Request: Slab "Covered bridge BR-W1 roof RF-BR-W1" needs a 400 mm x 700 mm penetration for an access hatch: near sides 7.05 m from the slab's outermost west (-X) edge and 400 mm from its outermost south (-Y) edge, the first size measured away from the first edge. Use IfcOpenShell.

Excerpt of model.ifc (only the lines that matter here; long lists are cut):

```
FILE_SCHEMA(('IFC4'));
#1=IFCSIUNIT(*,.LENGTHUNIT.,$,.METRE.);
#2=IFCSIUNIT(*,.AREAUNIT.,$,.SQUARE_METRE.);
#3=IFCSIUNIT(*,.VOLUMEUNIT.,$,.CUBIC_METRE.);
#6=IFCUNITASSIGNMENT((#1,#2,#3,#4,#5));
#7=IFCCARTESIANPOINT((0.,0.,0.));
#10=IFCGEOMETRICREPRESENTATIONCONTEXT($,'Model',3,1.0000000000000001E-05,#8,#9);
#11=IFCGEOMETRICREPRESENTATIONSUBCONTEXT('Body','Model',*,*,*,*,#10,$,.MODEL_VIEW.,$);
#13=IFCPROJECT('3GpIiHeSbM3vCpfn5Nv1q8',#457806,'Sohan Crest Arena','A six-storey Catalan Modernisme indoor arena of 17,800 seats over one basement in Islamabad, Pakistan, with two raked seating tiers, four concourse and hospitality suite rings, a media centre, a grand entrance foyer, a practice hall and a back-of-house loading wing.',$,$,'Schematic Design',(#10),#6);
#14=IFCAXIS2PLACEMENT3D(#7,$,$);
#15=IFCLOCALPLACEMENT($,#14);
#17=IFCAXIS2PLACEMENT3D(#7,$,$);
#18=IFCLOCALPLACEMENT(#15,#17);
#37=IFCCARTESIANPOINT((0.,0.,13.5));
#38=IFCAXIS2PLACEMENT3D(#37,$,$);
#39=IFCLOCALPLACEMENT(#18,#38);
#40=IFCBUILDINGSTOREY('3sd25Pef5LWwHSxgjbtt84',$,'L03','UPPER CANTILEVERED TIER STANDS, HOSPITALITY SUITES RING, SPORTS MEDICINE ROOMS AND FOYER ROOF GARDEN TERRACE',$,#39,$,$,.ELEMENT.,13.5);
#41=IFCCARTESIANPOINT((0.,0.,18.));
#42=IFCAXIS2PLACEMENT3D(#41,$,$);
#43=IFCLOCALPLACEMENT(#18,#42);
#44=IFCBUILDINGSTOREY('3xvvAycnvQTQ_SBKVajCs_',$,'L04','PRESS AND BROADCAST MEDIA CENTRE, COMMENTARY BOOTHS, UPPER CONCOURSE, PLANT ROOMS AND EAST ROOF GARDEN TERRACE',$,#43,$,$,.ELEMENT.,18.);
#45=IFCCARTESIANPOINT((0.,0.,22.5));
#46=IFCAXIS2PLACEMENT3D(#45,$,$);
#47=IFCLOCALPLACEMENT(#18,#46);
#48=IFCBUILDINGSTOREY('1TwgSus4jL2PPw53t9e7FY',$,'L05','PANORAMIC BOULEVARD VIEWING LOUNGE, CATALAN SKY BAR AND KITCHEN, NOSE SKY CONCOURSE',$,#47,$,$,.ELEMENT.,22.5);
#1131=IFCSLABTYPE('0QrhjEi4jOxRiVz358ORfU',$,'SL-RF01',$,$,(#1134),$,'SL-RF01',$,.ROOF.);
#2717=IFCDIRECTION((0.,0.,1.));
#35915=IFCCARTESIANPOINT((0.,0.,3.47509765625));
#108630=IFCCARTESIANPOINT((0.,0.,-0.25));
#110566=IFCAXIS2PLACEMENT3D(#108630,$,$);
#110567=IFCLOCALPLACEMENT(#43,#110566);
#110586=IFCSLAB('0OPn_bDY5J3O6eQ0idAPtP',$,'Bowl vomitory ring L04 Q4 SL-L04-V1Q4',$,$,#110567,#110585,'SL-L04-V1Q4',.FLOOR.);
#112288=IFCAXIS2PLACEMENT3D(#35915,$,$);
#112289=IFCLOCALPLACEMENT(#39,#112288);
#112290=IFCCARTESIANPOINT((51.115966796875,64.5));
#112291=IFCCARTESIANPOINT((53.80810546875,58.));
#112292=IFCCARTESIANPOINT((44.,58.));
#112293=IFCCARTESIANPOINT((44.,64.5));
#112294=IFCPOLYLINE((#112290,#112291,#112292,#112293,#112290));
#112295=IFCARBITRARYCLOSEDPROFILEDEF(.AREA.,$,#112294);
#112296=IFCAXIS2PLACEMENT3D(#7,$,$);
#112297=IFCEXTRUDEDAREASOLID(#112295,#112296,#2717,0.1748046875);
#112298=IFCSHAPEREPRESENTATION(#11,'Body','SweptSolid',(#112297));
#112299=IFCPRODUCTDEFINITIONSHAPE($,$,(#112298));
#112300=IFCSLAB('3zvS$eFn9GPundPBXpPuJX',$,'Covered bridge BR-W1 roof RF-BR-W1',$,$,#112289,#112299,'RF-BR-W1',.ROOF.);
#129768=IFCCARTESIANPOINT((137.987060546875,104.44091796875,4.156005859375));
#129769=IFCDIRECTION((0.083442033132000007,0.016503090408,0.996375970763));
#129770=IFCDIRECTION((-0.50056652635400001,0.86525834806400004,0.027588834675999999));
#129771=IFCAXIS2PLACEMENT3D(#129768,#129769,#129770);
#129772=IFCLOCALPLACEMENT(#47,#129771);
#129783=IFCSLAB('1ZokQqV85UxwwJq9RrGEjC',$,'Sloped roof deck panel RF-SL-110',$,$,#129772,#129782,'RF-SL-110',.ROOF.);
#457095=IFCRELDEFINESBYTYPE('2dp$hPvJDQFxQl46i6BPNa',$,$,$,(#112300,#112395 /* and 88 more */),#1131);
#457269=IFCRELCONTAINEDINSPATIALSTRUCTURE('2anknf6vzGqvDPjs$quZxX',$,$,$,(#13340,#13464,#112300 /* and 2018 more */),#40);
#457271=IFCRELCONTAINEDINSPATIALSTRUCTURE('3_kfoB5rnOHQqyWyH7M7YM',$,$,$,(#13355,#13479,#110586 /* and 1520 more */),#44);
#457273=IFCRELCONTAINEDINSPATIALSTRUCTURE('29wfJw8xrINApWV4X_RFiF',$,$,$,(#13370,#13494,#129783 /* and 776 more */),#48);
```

```python
import numpy as np
import ifcopenshell
import ifcopenshell.api.feature
import ifcopenshell.api.geometry
import ifcopenshell.api.root
import ifcopenshell.geom
import ifcopenshell.util.placement
import ifcopenshell.util.representation
import ifcopenshell.util.shape
import ifcopenshell.util.unit

model = ifcopenshell.open("model.ifc")
unit_scale = ifcopenshell.util.unit.calculate_unit_scale(model)
settings = ifcopenshell.geom.settings()


def volume(element):
    """Net volume in cubic metres, openings subtracted."""
    shape = ifcopenshell.geom.create_shape(settings, element)
    return ifcopenshell.util.shape.get_volume(shape.geometry)


slab = model.by_guid("3zvS$eFn9GPundPBXpPuJX")
before = volume(slab)

# Extent in the slab's own axes, in metres. The edges named are its -X and -Y sides.
slab_shape = ifcopenshell.geom.create_shape(settings, slab)
vertices = ifcopenshell.util.shape.get_vertices(slab_shape.geometry)
x_min, y_min, bottom = vertices.min(axis=0)
top = vertices[:, 2].max()

opening = ifcopenshell.api.root.create_entity(model, ifc_class="IfcOpeningElement", name="Access hatch opening", predefined_type="OPENING")
context = ifcopenshell.util.representation.get_context(model, "Model", "Body", "MODEL_VIEW")
width, depth = 0.4, 0.7
outline = [(0.0, 0.0), (width, 0.0), (width, depth), (0.0, depth), (0.0, 0.0)]
# Overshoot both faces by 50 mm so the cut is clean.
shape = ifcopenshell.api.geometry.add_slab_representation(
    model, context=context, depth=top - bottom + 0.1, polyline=outline
)
ifcopenshell.api.geometry.assign_representation(model, product=opening, representation=shape)

matrix = ifcopenshell.util.placement.get_local_placement(slab.ObjectPlacement)
matrix[:, 3] = matrix @ np.append(np.array([x_min + 7.05, y_min + 0.4, bottom - 0.05]) / unit_scale, 1.0)
ifcopenshell.api.geometry.edit_object_placement(model, product=opening, matrix=matrix, is_si=False)
ifcopenshell.api.feature.add_feature(model, feature=opening, element=slab)

after = volume(slab)

print(f"slab volume {before:.3f} -> {after:.3f} m3")

model.write("model_edited.ifc")
```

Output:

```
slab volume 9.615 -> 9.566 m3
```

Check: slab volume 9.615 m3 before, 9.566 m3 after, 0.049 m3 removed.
